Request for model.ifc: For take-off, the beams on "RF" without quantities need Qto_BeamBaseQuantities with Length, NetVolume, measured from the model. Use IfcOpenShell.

First a look at what the model holds.

```python
import ifcopenshell
import ifcopenshell.util.element
import ifcopenshell.util.unit

model = ifcopenshell.open("model.ifc")
print(model.schema)
for unit_type in ("LENGTHUNIT", "AREAUNIT", "VOLUMEUNIT"):
    print(unit_type, ifcopenshell.util.unit.calculate_unit_scale(model, unit_type))
storey = next(s for s in model.by_type("IfcBuildingStorey") if s.Name == "RF")
beams = [e for e in ifcopenshell.util.element.get_decomposition(storey) if e.is_a("IfcBeam")]
for e in sorted(beams, key=lambda e: e.id()):
    print(e.id(), e.is_a(), e.Name, list(ifcopenshell.util.element.get_psets(e, qtos_only=True)), sep=" | ")
```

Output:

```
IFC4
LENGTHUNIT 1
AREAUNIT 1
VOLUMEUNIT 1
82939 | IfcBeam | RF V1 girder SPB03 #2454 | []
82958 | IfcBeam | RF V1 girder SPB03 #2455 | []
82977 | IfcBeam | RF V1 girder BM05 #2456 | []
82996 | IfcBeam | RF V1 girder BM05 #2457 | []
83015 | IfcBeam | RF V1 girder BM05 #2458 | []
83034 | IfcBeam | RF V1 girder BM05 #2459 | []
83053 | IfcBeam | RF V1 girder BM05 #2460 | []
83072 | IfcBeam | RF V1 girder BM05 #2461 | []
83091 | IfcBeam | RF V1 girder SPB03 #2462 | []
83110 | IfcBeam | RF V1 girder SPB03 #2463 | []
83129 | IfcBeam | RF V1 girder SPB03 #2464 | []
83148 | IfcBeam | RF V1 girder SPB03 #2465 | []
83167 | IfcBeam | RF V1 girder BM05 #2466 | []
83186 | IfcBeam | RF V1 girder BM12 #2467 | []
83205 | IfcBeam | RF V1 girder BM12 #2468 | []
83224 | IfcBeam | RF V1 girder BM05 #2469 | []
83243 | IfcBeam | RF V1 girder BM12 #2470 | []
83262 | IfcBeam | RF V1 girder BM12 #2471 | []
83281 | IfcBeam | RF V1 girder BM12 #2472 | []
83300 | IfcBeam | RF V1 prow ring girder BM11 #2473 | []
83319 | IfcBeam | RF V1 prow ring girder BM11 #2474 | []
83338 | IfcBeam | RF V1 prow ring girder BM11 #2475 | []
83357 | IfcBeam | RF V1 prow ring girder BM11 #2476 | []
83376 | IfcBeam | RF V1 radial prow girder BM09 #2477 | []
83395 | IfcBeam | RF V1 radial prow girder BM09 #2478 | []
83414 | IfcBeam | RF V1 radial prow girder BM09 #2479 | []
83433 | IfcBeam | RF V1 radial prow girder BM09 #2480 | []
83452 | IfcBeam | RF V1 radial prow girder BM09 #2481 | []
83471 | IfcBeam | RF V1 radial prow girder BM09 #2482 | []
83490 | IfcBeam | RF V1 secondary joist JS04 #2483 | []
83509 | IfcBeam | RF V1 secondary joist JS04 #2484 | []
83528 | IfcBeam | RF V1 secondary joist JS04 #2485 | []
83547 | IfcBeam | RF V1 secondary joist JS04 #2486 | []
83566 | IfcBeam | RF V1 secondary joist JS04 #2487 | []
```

```python
import ifcopenshell
import ifcopenshell.api.pset
import ifcopenshell.geom
import ifcopenshell.util.element
import ifcopenshell.util.shape
import ifcopenshell.util.unit

model = ifcopenshell.open("model.ifc")
unit_scale = ifcopenshell.util.unit.calculate_unit_scale(model)
volume_scale = ifcopenshell.util.unit.calculate_unit_scale(model, "VOLUMEUNIT")
settings = ifcopenshell.geom.settings()

storey = next(s for s in model.by_type("IfcBuildingStorey") if s.Name == "RF")
beams = [e for e in ifcopenshell.util.element.get_decomposition(storey) if e.is_a("IfcBeam")]

for e in sorted(beams, key=lambda e: e.id()):
    if ifcopenshell.util.element.get_psets(e, qtos_only=True, should_inherit=False):
        continue
    # Geometry comes back in metres, in the element's own axes.
    shape = ifcopenshell.geom.create_shape(settings, e)
    values = {
        "Length": ifcopenshell.util.shape.get_max_xyz(shape.geometry) / unit_scale,
        "NetVolume": ifcopenshell.util.shape.get_volume(shape.geometry) / volume_scale,
    }
    qto = ifcopenshell.api.pset.add_qto(model, product=e, name="Qto_BeamBaseQuantities")
    ifcopenshell.api.pset.edit_qto(model, qto=qto, properties=values)
    print(e.id(), {k: round(v, 3) for k, v in values.items()})

model.write("model_rev.ifc")
```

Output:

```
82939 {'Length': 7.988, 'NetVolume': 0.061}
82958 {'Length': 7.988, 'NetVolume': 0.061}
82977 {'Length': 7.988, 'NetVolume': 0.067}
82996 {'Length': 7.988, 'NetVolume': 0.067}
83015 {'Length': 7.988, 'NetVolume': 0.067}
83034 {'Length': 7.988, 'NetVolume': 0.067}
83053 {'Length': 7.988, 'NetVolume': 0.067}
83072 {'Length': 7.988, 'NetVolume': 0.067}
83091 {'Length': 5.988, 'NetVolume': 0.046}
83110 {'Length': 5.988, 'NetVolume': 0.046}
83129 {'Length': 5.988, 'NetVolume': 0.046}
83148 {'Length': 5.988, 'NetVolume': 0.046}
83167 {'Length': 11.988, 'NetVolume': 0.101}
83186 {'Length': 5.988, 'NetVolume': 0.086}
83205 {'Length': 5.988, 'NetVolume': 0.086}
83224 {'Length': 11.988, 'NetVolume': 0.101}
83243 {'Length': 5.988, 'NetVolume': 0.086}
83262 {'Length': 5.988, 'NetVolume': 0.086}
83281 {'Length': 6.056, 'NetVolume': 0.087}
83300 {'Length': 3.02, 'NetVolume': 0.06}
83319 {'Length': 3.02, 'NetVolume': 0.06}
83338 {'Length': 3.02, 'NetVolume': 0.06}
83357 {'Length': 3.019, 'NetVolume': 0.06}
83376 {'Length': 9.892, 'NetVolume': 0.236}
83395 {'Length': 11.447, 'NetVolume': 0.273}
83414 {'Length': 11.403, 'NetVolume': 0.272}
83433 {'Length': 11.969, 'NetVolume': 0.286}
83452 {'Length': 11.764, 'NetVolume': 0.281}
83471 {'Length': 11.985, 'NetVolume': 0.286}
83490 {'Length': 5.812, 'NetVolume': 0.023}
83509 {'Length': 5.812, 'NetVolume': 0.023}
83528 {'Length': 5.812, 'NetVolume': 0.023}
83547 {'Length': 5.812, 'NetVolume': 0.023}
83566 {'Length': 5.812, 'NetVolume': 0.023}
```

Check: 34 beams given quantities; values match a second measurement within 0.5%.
